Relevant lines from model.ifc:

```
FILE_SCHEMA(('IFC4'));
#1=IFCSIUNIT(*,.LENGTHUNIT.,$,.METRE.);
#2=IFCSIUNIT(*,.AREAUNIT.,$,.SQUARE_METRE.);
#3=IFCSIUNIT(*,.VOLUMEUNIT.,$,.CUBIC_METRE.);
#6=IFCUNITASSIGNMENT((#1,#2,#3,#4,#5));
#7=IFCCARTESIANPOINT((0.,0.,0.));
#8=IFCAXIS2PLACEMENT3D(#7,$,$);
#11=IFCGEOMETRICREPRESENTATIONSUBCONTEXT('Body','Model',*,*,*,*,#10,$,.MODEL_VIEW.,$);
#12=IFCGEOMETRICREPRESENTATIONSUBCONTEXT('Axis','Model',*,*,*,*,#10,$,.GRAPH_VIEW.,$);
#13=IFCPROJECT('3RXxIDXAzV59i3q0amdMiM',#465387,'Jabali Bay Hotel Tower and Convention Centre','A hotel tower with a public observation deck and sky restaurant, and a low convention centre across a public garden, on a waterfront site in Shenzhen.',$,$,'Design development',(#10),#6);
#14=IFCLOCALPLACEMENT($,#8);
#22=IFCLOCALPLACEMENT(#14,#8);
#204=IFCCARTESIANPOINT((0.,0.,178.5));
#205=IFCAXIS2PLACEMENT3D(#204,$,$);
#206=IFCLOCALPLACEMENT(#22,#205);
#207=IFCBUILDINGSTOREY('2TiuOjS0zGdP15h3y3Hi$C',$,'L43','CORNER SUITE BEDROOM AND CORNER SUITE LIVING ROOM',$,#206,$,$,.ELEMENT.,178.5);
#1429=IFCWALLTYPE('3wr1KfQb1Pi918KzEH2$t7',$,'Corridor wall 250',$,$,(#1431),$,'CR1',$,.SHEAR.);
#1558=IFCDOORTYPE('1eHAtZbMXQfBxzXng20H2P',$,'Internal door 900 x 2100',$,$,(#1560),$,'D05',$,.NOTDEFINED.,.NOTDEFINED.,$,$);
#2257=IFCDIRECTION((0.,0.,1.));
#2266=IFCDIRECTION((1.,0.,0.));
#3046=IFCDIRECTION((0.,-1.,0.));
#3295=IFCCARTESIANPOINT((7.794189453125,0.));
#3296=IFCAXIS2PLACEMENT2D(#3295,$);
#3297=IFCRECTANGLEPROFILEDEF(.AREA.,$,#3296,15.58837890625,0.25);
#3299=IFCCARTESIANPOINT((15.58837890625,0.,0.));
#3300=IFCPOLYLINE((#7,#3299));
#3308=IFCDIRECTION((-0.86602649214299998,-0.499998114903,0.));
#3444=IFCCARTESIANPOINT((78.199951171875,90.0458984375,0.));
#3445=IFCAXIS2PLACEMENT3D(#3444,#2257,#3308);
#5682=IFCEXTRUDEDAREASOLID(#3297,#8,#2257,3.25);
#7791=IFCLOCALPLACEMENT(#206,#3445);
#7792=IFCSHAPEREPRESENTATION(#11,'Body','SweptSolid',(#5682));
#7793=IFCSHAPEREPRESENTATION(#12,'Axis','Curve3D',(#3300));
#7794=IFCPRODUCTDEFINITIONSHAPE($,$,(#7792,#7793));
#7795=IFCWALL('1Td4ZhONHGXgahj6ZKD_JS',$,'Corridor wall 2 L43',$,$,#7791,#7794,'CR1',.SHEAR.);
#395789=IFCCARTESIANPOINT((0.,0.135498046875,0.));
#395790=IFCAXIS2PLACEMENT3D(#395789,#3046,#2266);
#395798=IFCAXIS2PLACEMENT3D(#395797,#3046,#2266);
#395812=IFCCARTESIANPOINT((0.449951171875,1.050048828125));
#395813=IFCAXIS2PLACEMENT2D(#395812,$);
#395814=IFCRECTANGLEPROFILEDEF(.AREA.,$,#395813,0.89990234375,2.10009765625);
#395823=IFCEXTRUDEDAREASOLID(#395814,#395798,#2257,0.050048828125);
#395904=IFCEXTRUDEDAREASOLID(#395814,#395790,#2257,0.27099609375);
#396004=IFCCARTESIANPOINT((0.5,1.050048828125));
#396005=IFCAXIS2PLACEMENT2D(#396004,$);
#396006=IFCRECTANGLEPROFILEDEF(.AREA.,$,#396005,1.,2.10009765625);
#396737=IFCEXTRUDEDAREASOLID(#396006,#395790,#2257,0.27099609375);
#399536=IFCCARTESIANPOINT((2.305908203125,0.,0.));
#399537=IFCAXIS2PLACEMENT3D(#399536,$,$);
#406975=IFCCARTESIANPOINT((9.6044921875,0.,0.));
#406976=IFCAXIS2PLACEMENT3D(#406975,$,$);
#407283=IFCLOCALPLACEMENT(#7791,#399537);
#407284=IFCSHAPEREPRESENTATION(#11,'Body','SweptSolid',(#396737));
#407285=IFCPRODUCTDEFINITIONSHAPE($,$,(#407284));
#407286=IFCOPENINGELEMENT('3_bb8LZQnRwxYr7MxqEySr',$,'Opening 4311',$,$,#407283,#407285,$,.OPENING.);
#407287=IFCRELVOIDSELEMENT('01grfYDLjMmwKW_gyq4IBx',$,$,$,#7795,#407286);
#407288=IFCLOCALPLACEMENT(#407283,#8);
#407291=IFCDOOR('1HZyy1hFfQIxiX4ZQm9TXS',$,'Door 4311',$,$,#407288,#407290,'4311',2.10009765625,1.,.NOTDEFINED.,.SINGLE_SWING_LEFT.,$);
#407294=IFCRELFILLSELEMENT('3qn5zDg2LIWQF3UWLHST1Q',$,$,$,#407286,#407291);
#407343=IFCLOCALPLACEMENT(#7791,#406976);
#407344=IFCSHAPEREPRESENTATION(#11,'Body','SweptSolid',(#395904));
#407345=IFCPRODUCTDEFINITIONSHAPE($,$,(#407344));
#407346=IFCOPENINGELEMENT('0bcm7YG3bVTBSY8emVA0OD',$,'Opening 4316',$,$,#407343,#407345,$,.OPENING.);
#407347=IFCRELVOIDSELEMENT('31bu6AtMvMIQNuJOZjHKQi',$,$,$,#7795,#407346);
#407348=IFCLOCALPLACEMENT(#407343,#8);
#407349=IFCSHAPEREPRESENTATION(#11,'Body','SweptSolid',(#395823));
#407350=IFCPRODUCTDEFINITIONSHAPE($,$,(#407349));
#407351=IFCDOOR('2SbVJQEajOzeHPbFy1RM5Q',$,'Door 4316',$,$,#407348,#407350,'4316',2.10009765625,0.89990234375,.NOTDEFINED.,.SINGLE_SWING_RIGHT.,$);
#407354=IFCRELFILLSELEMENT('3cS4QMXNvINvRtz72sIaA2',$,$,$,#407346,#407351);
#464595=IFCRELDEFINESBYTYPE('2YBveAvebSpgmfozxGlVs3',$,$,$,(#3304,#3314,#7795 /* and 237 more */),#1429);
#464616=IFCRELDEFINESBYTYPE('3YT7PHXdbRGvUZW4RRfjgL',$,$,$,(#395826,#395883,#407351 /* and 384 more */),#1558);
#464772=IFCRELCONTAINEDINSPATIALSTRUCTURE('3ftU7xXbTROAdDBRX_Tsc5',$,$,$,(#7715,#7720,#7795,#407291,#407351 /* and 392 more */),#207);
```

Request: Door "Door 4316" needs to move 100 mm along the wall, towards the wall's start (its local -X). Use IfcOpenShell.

```python
import ifcopenshell
import ifcopenshell.api.geometry
import ifcopenshell.util.placement

model = ifcopenshell.open("model.ifc")

door = model.by_guid("2SbVJQEajOzeHPbFy1RM5Q")
opening = door.FillsVoids[0].RelatingOpeningElement
wall = opening.VoidsElements[0].RelatingBuildingElement

wall_matrix = ifcopenshell.util.placement.get_local_placement(wall.ObjectPlacement)
shift = wall_matrix[:3, 0] * -0.1
before = ifcopenshell.util.placement.get_local_placement(door.ObjectPlacement)[:3, 3].copy()

# The door is placed relative to its opening, so it follows when the opening moves.
matrix = ifcopenshell.util.placement.get_local_placement(opening.ObjectPlacement)
matrix[:3, 3] += shift
ifcopenshell.api.geometry.edit_object_placement(
    model, product=opening, matrix=matrix, is_si=False, should_transform_children=True
)

after = ifcopenshell.util.placement.get_local_placement(door.ObjectPlacement)[:3, 3]
print("door moved by", (after - before).round(3) + 0.0)

model.write("model_rev.ifc")
```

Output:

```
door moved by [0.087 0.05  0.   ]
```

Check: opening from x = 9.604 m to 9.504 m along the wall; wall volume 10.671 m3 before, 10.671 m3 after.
